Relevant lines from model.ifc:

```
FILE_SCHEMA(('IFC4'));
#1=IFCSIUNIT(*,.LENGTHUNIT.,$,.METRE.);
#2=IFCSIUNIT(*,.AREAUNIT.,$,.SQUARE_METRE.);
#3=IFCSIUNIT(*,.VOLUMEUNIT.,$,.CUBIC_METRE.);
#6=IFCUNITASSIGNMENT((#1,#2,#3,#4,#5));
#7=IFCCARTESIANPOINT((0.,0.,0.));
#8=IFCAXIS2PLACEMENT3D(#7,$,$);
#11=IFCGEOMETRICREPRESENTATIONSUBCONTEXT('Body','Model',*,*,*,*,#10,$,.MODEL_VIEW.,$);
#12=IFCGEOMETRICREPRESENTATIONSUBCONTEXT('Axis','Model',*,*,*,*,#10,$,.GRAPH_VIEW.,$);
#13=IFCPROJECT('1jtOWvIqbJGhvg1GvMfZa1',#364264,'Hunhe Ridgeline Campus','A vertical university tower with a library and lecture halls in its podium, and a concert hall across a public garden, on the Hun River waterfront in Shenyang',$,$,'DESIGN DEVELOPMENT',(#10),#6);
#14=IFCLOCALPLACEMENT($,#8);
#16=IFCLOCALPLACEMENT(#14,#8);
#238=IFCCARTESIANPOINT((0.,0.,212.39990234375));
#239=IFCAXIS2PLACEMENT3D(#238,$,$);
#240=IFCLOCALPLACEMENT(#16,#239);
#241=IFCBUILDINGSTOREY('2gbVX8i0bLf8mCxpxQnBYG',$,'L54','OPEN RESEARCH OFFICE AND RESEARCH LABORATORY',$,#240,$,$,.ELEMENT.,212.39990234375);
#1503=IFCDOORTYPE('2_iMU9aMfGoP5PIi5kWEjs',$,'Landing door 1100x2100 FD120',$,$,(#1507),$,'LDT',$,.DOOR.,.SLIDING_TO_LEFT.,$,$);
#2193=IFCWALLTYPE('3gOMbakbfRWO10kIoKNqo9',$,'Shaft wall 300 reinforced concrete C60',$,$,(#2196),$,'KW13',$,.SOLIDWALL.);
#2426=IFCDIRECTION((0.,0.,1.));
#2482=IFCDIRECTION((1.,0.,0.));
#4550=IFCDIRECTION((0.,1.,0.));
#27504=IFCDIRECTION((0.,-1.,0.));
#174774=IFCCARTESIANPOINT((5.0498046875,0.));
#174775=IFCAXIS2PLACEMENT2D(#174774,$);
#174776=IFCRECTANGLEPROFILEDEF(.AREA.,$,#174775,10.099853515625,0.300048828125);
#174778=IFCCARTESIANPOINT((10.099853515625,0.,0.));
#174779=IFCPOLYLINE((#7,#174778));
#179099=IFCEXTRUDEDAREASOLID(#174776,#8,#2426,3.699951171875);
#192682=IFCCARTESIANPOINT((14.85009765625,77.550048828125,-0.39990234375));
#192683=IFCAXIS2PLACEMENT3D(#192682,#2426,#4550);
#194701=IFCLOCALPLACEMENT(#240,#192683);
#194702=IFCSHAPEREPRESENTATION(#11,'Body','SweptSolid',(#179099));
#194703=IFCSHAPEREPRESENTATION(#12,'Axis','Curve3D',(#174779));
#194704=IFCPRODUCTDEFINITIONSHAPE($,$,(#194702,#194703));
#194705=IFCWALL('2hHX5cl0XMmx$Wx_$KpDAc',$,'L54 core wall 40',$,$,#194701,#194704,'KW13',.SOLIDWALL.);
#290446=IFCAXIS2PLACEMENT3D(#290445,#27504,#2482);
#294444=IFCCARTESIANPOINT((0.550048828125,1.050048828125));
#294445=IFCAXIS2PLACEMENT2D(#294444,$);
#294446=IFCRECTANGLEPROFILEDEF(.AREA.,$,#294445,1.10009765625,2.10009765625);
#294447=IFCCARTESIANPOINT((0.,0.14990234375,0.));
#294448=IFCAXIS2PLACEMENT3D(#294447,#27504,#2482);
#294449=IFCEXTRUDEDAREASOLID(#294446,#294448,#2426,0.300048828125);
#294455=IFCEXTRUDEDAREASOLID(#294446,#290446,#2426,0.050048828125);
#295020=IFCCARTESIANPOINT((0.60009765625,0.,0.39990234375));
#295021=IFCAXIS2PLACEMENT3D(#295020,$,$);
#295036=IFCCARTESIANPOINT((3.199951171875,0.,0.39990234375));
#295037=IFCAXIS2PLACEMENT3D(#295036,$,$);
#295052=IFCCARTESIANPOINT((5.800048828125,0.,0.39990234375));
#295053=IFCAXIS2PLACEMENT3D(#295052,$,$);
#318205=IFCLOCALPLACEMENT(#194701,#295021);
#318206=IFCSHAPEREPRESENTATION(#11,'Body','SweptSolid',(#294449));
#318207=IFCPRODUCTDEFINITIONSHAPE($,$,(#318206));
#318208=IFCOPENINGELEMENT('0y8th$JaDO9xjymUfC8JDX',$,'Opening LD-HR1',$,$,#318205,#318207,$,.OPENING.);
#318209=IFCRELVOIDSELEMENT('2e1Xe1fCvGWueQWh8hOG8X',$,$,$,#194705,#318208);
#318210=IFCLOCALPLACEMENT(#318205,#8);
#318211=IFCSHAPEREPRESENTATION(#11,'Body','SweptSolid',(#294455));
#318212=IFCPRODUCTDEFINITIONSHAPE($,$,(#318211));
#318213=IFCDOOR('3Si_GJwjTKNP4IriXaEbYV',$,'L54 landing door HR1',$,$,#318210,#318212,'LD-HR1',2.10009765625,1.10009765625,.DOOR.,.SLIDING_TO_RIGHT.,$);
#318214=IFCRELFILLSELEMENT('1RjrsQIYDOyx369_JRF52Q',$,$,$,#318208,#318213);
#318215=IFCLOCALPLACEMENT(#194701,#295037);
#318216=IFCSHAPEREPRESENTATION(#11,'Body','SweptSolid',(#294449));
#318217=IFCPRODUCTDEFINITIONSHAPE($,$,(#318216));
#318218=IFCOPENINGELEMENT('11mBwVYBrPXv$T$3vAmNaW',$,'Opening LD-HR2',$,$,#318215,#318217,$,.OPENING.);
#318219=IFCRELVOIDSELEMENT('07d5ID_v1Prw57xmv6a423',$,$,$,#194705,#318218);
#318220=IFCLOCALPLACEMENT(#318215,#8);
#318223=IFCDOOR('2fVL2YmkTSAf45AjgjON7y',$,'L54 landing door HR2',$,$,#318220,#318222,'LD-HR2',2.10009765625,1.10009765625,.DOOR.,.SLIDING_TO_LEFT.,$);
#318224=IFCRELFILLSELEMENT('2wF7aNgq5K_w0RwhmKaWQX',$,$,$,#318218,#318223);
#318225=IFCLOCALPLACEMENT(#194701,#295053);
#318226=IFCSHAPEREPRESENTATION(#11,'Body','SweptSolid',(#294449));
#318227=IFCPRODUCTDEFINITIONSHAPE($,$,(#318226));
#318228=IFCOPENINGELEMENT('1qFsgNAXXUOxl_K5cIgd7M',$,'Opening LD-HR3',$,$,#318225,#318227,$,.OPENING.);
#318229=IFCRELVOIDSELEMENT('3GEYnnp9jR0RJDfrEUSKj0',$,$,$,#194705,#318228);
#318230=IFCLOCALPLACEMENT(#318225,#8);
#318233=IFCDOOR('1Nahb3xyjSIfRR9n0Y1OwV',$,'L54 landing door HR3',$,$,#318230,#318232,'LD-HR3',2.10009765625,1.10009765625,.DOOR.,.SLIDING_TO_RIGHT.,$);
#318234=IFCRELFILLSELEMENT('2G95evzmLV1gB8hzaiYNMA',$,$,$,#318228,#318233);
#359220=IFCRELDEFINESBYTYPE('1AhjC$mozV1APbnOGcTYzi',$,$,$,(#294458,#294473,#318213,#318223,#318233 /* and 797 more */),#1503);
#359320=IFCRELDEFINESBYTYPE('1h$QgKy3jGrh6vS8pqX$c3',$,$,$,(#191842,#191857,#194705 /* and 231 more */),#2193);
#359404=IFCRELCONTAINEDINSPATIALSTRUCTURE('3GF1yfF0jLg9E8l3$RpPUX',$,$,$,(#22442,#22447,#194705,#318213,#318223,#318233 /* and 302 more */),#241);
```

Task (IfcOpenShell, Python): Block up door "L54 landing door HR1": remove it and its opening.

```python
import ifcopenshell
import ifcopenshell.api.feature
import ifcopenshell.api.root
import ifcopenshell.geom
import ifcopenshell.util.shape

model = ifcopenshell.open("model.ifc")
settings = ifcopenshell.geom.settings()


def volume(element):
    """Net volume in cubic metres, openings subtracted."""
    shape = ifcopenshell.geom.create_shape(settings, element)
    return ifcopenshell.util.shape.get_volume(shape.geometry)


door = model.by_id(318213)
opening = door.FillsVoids[0].RelatingOpeningElement
wall = opening.VoidsElements[0].RelatingBuildingElement
before = volume(wall)

ifcopenshell.api.root.remove_product(model, product=door)
ifcopenshell.api.feature.remove_feature(model, feature=opening)

after = volume(wall)

print(f"wall volume {before:.3f} -> {after:.3f} m3")

model.write("model_updated.ifc")
```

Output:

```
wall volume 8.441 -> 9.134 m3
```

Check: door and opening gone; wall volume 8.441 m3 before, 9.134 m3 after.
